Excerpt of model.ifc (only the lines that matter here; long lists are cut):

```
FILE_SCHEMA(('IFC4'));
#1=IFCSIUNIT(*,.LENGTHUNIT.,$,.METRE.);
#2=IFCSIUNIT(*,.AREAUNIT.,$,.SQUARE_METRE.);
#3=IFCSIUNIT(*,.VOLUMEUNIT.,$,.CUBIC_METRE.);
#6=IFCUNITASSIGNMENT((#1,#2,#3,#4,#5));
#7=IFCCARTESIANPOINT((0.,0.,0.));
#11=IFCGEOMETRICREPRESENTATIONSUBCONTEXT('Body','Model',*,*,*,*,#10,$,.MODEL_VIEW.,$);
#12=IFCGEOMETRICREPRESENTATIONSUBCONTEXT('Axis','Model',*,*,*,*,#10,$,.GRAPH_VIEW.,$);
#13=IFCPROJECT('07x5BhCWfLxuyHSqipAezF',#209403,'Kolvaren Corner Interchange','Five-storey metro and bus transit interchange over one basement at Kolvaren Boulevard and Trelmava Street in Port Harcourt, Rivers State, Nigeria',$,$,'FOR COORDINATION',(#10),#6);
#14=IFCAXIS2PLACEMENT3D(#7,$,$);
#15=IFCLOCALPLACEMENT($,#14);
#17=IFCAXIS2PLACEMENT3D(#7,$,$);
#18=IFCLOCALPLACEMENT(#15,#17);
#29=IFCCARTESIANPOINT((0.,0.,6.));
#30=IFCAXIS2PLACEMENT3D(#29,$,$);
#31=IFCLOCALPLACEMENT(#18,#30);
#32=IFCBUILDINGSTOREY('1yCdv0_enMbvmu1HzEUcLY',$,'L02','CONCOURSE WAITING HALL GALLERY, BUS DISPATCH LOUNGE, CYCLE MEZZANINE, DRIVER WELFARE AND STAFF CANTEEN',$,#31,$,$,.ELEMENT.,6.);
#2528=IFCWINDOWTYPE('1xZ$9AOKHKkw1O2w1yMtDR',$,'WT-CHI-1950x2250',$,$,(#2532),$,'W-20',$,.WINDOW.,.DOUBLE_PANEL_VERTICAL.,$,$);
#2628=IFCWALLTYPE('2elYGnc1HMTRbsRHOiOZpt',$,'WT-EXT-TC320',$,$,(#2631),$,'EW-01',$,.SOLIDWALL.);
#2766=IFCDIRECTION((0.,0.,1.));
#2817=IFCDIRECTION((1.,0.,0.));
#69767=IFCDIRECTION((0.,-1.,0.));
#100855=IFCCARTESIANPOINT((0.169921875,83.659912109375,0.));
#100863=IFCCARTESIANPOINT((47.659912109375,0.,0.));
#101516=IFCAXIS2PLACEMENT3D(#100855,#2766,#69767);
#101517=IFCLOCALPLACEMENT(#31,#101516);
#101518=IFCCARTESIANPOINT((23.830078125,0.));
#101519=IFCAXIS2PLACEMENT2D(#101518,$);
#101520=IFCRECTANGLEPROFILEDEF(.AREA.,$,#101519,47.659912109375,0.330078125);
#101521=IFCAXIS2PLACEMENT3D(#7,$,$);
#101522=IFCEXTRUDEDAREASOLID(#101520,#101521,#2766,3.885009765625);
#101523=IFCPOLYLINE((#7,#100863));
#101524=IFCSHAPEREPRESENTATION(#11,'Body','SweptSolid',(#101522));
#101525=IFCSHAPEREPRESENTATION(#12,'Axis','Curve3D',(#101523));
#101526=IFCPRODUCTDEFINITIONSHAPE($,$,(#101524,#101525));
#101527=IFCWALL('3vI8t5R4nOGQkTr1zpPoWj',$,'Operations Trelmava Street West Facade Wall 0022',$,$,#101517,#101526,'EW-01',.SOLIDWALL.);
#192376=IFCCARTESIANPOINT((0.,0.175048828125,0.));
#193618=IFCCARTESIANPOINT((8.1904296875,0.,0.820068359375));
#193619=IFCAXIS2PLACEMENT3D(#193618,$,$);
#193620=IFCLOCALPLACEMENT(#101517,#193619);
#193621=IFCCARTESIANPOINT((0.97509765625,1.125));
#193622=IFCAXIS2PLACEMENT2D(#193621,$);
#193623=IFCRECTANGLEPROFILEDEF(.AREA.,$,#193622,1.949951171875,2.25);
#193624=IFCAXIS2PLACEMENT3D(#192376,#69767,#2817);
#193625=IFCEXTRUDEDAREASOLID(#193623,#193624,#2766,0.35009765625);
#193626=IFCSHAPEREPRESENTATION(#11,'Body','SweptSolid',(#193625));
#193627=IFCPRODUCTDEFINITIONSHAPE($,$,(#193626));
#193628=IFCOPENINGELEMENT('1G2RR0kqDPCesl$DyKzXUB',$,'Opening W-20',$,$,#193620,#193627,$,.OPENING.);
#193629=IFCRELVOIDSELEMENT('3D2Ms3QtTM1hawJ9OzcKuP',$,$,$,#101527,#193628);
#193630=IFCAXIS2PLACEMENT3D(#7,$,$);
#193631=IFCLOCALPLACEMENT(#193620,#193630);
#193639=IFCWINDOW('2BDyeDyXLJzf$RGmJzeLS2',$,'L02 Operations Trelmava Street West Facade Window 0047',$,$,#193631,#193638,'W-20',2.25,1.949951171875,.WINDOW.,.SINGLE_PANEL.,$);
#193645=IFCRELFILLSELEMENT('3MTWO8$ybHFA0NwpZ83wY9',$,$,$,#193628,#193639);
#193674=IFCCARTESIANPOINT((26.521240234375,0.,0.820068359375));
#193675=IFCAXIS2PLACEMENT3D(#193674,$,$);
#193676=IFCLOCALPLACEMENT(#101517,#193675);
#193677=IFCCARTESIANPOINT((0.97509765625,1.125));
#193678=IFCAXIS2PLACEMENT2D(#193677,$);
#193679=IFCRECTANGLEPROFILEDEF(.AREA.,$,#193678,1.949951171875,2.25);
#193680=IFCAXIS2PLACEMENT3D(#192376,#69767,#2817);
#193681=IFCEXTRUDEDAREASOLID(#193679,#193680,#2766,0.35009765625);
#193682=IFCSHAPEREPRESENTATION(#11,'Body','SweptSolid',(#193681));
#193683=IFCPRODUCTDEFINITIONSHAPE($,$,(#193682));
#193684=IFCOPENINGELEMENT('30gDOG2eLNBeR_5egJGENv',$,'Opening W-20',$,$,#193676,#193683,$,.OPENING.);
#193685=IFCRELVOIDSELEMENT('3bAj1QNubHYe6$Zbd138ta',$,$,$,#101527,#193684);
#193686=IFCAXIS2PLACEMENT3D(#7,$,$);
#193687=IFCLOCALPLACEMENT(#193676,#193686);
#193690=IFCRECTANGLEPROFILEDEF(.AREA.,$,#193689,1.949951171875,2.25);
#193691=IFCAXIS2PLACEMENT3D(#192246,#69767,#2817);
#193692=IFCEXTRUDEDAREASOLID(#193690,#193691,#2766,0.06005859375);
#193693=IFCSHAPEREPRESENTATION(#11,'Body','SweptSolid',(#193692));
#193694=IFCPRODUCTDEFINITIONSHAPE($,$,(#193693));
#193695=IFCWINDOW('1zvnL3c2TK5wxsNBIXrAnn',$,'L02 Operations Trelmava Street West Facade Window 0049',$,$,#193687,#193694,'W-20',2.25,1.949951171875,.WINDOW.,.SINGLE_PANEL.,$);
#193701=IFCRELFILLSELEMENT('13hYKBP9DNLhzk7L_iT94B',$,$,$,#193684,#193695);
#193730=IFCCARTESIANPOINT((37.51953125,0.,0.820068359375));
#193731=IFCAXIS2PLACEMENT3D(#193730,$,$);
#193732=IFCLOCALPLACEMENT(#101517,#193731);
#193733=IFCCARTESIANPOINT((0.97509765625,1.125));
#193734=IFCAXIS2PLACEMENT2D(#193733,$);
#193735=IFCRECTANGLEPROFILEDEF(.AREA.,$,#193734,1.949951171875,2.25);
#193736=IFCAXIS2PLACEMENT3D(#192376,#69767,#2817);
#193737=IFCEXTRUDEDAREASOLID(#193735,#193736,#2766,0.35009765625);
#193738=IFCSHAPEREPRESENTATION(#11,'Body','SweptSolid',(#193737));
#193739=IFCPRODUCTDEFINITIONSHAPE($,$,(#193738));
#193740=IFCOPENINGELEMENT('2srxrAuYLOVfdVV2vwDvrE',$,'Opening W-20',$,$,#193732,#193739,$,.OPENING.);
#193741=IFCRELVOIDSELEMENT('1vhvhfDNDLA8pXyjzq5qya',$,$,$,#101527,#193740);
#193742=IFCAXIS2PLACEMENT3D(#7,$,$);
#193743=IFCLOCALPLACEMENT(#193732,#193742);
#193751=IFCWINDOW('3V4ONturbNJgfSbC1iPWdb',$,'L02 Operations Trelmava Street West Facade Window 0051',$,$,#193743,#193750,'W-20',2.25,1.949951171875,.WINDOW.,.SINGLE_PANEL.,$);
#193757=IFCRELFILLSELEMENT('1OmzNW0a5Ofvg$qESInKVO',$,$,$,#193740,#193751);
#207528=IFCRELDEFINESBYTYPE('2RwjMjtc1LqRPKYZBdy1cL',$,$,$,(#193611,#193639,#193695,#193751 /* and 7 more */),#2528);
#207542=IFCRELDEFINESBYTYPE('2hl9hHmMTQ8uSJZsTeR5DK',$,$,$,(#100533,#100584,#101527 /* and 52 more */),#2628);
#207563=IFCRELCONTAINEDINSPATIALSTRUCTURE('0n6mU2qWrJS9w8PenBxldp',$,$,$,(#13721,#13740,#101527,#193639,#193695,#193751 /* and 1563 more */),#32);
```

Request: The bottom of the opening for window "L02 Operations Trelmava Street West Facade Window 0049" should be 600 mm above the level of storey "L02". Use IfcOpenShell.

```python
import numpy as np
import ifcopenshell
import ifcopenshell.api.geometry
import ifcopenshell.geom
import ifcopenshell.util.element
import ifcopenshell.util.placement
import ifcopenshell.util.shape
import ifcopenshell.util.unit

model = ifcopenshell.open("model.ifc")
unit_scale = ifcopenshell.util.unit.calculate_unit_scale(model)

window = model.by_guid("1zvnL3c2TK5wxsNBIXrAnn")
opening = window.FillsVoids[0].RelatingOpeningElement
storey = ifcopenshell.util.element.get_container(window, ifc_class="IfcBuildingStorey")
level = ifcopenshell.util.placement.get_local_placement(storey.ObjectPlacement)[2, 3]

# The opening's origin need not be at the sill, so measure its lowest point.
shape = ifcopenshell.geom.create_shape(ifcopenshell.geom.settings(), opening)
bottom = ifcopenshell.util.shape.get_shape_bottom_elevation(shape, shape.geometry) / unit_scale
dz = level + 0.6 / unit_scale - bottom

shift = np.array([0.0, 0.0, dz])
# The window is placed relative to its opening, so it follows when the opening moves.
matrix = ifcopenshell.util.placement.get_local_placement(opening.ObjectPlacement)
matrix[:3, 3] += shift
ifcopenshell.api.geometry.edit_object_placement(
    model, product=opening, matrix=matrix, is_si=False, should_transform_children=True
)

print(f"moved by {dz * unit_scale:+.3f} m")

model.write("model_rev.ifc")
```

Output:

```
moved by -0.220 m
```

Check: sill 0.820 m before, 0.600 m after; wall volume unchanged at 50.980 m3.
